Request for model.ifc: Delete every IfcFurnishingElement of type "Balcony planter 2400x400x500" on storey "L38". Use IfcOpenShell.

First a look at what the model holds.

```python
import ifcopenshell
import ifcopenshell.util.element

model = ifcopenshell.open("model.ifc")
print(model.schema)
storey = next(s for s in model.by_type("IfcBuildingStorey") if s.Name == "L38")
furniture = [e for e in ifcopenshell.util.element.get_decomposition(storey) if e.is_a("IfcFurnishingElement")]
seen = {}
for e in furniture:
    element_type = ifcopenshell.util.element.get_type(e)
    name = element_type.Name if element_type not in (None, e) else None
    seen[name] = seen.get(name, 0) + 1
for name, count in sorted(seen.items(), key=str):
    print(count, "x", name)
```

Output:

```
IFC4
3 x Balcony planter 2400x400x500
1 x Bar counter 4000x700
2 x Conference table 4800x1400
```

```python
import ifcopenshell
import ifcopenshell.api.root
import ifcopenshell.util.element

model = ifcopenshell.open("model.ifc")

storey = next(s for s in model.by_type("IfcBuildingStorey") if s.Name == "L38")
furniture = [e for e in ifcopenshell.util.element.get_decomposition(storey) if e.is_a("IfcFurnishingElement")]
targets = [e for e in furniture if (t := ifcopenshell.util.element.get_type(e)) not in (None, e) and t.Name == "Balcony planter 2400x400x500"]

for e in targets:
    ifcopenshell.api.root.remove_product(model, product=e)
print(len(targets), "removed")

model.write("model_v2.ifc")
```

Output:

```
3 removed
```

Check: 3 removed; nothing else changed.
